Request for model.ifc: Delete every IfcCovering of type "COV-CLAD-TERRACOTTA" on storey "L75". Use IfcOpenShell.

First a look at what the model holds.

```python
import ifcopenshell
import ifcopenshell.util.element

model = ifcopenshell.open("model.ifc")
print(model.schema)
storey = next(s for s in model.by_type("IfcBuildingStorey") if s.Name == "L75")
coverings = [e for e in ifcopenshell.util.element.get_decomposition(storey) if e.is_a("IfcCovering")]
seen = {}
for e in coverings:
    element_type = ifcopenshell.util.element.get_type(e)
    name = element_type.Name if element_type not in (None, e) else None
    seen[name] = seen.get(name, 0) + 1
for name, count in sorted(seen.items(), key=str):
    print(count, "x", name)
```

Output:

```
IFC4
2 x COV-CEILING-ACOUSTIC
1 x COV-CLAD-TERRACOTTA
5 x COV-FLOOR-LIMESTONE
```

```python
import ifcopenshell
import ifcopenshell.api.root
import ifcopenshell.util.element

model = ifcopenshell.open("model.ifc")

storey = next(s for s in model.by_type("IfcBuildingStorey") if s.Name == "L75")
coverings = [e for e in ifcopenshell.util.element.get_decomposition(storey) if e.is_a("IfcCovering")]
targets = [e for e in coverings if (t := ifcopenshell.util.element.get_type(e)) not in (None, e) and t.Name == "COV-CLAD-TERRACOTTA"]

for e in targets:
    ifcopenshell.api.root.remove_product(model, product=e)
print(len(targets), "removed")

model.write("model_rev.ifc")
```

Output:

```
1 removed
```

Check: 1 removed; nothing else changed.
